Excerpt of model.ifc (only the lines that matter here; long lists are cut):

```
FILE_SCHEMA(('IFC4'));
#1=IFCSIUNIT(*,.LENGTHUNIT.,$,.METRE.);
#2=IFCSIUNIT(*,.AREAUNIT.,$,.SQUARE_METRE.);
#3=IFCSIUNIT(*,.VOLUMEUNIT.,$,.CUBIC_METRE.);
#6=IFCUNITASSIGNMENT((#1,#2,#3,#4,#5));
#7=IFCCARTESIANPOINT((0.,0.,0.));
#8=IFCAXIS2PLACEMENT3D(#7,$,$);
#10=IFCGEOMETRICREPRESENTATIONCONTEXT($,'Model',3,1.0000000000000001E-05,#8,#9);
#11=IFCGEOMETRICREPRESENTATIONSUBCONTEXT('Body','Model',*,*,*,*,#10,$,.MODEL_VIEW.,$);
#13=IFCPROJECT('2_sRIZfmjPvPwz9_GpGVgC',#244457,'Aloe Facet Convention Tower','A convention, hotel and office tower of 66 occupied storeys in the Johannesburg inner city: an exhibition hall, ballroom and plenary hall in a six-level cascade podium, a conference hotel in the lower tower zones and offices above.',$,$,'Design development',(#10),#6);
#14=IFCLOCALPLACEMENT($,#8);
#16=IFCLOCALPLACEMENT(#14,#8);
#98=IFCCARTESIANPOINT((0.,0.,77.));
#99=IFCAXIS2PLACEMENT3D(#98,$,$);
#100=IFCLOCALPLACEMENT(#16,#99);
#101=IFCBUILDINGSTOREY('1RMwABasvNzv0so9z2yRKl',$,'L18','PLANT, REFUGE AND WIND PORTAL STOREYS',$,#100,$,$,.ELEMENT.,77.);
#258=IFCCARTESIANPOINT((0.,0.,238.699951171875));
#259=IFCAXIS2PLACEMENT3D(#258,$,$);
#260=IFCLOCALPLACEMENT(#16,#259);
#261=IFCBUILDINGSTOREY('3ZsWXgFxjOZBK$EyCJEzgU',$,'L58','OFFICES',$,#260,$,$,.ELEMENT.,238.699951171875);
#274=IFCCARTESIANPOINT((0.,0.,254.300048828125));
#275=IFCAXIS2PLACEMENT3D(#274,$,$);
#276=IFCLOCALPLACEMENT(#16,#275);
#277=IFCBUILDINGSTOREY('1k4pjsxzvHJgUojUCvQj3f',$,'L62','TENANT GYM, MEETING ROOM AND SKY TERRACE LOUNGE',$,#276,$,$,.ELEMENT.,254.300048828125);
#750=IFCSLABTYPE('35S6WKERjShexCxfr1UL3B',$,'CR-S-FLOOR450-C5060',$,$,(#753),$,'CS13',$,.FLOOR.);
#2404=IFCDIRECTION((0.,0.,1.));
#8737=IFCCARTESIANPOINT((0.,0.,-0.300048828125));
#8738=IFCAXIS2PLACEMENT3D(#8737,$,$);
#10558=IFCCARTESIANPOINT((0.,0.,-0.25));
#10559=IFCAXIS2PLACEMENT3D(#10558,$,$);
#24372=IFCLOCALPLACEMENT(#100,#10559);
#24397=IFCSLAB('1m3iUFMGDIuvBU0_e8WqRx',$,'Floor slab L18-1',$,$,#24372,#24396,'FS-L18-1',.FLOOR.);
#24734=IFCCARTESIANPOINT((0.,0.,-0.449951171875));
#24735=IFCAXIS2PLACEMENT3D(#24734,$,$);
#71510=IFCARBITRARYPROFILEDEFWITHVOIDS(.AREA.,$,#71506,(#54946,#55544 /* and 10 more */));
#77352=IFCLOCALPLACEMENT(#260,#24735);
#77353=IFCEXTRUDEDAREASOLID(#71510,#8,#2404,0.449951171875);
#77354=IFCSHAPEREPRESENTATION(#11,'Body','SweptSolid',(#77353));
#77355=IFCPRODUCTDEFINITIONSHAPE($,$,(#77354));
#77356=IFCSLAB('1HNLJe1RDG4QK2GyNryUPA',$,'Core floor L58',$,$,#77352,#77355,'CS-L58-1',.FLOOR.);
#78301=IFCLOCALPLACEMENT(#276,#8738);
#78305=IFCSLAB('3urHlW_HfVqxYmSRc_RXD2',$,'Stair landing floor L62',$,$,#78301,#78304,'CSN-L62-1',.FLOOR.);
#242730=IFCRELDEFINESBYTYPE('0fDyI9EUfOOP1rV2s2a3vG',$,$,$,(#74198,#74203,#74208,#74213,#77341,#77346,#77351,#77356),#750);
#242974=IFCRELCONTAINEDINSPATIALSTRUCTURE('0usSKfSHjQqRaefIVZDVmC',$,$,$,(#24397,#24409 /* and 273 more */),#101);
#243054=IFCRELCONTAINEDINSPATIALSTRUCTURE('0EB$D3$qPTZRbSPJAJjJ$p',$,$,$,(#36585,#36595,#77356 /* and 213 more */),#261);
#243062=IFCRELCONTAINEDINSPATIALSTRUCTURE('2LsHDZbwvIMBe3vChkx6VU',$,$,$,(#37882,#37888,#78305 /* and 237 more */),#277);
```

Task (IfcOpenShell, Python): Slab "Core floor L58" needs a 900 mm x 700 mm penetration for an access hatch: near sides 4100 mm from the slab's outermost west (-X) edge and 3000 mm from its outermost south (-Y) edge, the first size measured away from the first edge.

```python
import numpy as np
import ifcopenshell
import ifcopenshell.api.feature
import ifcopenshell.api.geometry
import ifcopenshell.api.root
import ifcopenshell.geom
import ifcopenshell.util.placement
import ifcopenshell.util.representation
import ifcopenshell.util.shape
import ifcopenshell.util.unit

model = ifcopenshell.open("model.ifc")
unit_scale = ifcopenshell.util.unit.calculate_unit_scale(model)
settings = ifcopenshell.geom.settings()


def volume(element):
    """Net volume in cubic metres, openings subtracted."""
    shape = ifcopenshell.geom.create_shape(settings, element)
    return ifcopenshell.util.shape.get_volume(shape.geometry)


slab = model.by_id(77356)
before = volume(slab)

# Extent in the slab's own axes, in metres. The edges named are its -X and -Y sides.
slab_shape = ifcopenshell.geom.create_shape(settings, slab)
vertices = ifcopenshell.util.shape.get_vertices(slab_shape.geometry)
x_min, y_min, bottom = vertices.min(axis=0)
top = vertices[:, 2].max()

opening = ifcopenshell.api.root.create_entity(model, ifc_class="IfcOpeningElement", name="Access hatch opening", predefined_type="OPENING")
context = ifcopenshell.util.representation.get_context(model, "Model", "Body", "MODEL_VIEW")
width, depth = 0.9, 0.7
outline = [(0.0, 0.0), (width, 0.0), (width, depth), (0.0, depth), (0.0, 0.0)]
# Overshoot both faces by 50 mm so the cut is clean.
shape = ifcopenshell.api.geometry.add_slab_representation(
    model, context=context, depth=top - bottom + 0.1, polyline=outline
)
ifcopenshell.api.geometry.assign_representation(model, product=opening, representation=shape)

matrix = ifcopenshell.util.placement.get_local_placement(slab.ObjectPlacement)
matrix[:, 3] = matrix @ np.append(np.array([x_min + 4.1, y_min + 3, bottom - 0.05]) / unit_scale, 1.0)
ifcopenshell.api.geometry.edit_object_placement(model, product=opening, matrix=matrix, is_si=False)
ifcopenshell.api.feature.add_feature(model, feature=opening, element=slab)

after = volume(slab)

print(f"slab volume {before:.3f} -> {after:.3f} m3")

model.write("model_edited.ifc")
```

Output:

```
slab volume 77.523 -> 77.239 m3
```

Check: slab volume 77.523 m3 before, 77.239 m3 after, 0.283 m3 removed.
